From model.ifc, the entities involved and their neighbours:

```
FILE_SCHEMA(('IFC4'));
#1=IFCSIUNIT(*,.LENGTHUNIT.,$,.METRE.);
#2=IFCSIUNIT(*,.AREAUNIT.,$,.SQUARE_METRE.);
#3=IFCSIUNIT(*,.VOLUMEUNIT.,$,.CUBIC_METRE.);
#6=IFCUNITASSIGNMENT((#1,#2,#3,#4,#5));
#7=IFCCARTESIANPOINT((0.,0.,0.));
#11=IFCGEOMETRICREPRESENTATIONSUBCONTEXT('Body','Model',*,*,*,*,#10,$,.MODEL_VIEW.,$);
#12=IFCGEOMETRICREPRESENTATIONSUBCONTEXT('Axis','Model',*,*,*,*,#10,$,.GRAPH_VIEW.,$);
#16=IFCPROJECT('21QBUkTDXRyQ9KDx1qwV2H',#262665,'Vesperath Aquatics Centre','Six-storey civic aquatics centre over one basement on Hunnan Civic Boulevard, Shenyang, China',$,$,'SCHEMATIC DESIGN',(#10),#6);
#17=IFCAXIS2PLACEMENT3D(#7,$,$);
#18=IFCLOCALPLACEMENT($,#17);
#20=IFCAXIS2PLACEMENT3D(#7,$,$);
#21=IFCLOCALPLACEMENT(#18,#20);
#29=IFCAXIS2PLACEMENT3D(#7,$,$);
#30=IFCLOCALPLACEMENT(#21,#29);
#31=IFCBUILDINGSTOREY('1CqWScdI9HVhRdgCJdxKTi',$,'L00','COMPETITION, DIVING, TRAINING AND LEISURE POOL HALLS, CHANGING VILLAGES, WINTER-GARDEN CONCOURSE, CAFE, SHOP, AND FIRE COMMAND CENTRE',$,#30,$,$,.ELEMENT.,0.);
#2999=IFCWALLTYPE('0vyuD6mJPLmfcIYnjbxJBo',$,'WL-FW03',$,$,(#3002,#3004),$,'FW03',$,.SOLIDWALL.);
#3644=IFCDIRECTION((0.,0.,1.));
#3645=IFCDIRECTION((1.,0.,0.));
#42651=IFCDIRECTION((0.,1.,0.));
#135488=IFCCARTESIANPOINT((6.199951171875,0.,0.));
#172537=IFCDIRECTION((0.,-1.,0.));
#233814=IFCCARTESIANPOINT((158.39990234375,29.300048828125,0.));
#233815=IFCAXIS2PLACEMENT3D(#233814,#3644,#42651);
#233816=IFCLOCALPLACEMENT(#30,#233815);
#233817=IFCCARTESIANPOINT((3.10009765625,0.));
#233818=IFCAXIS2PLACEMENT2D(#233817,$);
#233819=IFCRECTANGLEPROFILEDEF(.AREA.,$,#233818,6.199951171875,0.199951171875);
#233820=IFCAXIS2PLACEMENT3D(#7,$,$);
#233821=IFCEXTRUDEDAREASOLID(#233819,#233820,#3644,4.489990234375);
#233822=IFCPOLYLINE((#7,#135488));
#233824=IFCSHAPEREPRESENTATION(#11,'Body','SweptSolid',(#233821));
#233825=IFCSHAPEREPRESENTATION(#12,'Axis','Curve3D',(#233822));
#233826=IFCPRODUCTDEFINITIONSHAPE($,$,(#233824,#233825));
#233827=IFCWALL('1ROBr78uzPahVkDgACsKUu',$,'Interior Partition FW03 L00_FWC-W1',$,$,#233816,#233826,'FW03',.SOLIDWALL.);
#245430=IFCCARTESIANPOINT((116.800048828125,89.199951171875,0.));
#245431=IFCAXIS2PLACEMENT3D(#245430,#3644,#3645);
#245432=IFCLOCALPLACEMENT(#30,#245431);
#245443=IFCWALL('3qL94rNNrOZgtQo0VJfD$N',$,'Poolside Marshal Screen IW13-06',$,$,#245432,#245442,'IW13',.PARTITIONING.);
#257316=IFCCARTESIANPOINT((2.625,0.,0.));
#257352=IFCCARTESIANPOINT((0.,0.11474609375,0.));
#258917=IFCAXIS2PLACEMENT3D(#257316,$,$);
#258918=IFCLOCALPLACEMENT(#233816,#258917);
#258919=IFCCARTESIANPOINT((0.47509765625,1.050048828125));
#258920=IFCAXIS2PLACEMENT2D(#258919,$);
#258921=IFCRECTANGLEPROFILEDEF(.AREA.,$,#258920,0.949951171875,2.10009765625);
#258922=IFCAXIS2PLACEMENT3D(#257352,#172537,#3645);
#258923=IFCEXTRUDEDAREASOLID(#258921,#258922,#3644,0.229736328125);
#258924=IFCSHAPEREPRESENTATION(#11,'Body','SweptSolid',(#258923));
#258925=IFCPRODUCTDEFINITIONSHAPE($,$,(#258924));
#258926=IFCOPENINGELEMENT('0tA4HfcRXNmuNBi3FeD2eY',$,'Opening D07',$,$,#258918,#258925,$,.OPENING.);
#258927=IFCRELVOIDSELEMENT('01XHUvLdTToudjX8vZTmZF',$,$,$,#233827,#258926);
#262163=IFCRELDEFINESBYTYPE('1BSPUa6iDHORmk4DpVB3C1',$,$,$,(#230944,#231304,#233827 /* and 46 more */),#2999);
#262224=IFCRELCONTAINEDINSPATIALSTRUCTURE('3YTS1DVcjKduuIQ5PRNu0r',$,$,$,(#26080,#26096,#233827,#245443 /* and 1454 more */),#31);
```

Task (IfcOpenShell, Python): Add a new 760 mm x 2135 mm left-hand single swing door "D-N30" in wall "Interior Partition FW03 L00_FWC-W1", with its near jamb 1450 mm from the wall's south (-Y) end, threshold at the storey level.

```python
import numpy as np
import ifcopenshell
import ifcopenshell.api.feature
import ifcopenshell.api.geometry
import ifcopenshell.api.root
import ifcopenshell.api.spatial
import ifcopenshell.geom
import ifcopenshell.util.element
import ifcopenshell.util.placement
import ifcopenshell.util.representation
import ifcopenshell.util.shape
import ifcopenshell.util.unit

model = ifcopenshell.open("model.ifc")
unit_scale = ifcopenshell.util.unit.calculate_unit_scale(model)
settings = ifcopenshell.geom.settings()


def volume(element):
    """Net volume in cubic metres, openings subtracted."""
    shape = ifcopenshell.geom.create_shape(settings, element)
    return ifcopenshell.util.shape.get_volume(shape.geometry)


wall = model.by_id(233827)
storey = ifcopenshell.util.element.get_container(wall, ifc_class="IfcBuildingStorey")
context = ifcopenshell.util.representation.get_context(model, "Model", "Body", "MODEL_VIEW")
before = volume(wall)

width, height, from_end, sill = 0.76, 2.135, 1.45, 0.0  # metres

# The wall runs along its own X axis, and the end named is its -X end.
wall_shape = ifcopenshell.geom.create_shape(settings, wall)
x, y, z = ifcopenshell.util.shape.get_vertices(wall_shape.geometry).T
start = x.min() + from_end
face, thickness = float(y.min()), float(y.max() - y.min())
wall_matrix = ifcopenshell.util.placement.get_local_placement(wall.ObjectPlacement)
level = ifcopenshell.util.placement.get_local_placement(storey.ObjectPlacement)[2, 3]


def in_wall(x, y):
    """Placement at x, y metres in the wall's axes, at sill height."""
    matrix = wall_matrix.copy()
    matrix[:, 3] = wall_matrix @ np.array([x / unit_scale, y / unit_scale, 0.0, 1.0])
    matrix[2, 3] = level + sill / unit_scale
    return matrix


# Opening: a box that overshoots both wall faces by 50 mm.
opening = ifcopenshell.api.root.create_entity(model, ifc_class="IfcOpeningElement", predefined_type="OPENING")
box = ifcopenshell.api.geometry.add_wall_representation(
    model, context=context, length=width, height=height, thickness=thickness + 0.1
)
ifcopenshell.api.geometry.assign_representation(model, product=opening, representation=box)
ifcopenshell.api.geometry.edit_object_placement(model, product=opening, matrix=in_wall(start, face - 0.05), is_si=False)
ifcopenshell.api.feature.add_feature(model, feature=opening, element=wall)

door = ifcopenshell.api.root.create_entity(model, ifc_class="IfcDoor", name="D-N30", predefined_type="DOOR")
door.OverallWidth, door.OverallHeight = width / unit_scale, height / unit_scale
door.OperationType = "SINGLE_SWING_LEFT"
body = ifcopenshell.api.geometry.add_door_representation(
    model,
    context=context,
    overall_width=door.OverallWidth,
    overall_height=door.OverallHeight,
    operation_type="SINGLE_SWING_LEFT",
    lining_properties={"LiningDepth": thickness / unit_scale, "ThresholdDepth": thickness / unit_scale},
)
ifcopenshell.api.geometry.assign_representation(model, product=door, representation=body)
ifcopenshell.api.spatial.assign_container(model, products=[door], relating_structure=storey)
ifcopenshell.api.feature.add_filling(model, opening=opening, element=door)

# The lining spans the wall, so the door starts at the wall face.
ifcopenshell.api.geometry.edit_object_placement(model, product=door, matrix=in_wall(start, face), is_si=False)

after = volume(wall)

print(f"wall volume {before:.3f} -> {after:.3f} m3")

model.write("model-out.ifc")
```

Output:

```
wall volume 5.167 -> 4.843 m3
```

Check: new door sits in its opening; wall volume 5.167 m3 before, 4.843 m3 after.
